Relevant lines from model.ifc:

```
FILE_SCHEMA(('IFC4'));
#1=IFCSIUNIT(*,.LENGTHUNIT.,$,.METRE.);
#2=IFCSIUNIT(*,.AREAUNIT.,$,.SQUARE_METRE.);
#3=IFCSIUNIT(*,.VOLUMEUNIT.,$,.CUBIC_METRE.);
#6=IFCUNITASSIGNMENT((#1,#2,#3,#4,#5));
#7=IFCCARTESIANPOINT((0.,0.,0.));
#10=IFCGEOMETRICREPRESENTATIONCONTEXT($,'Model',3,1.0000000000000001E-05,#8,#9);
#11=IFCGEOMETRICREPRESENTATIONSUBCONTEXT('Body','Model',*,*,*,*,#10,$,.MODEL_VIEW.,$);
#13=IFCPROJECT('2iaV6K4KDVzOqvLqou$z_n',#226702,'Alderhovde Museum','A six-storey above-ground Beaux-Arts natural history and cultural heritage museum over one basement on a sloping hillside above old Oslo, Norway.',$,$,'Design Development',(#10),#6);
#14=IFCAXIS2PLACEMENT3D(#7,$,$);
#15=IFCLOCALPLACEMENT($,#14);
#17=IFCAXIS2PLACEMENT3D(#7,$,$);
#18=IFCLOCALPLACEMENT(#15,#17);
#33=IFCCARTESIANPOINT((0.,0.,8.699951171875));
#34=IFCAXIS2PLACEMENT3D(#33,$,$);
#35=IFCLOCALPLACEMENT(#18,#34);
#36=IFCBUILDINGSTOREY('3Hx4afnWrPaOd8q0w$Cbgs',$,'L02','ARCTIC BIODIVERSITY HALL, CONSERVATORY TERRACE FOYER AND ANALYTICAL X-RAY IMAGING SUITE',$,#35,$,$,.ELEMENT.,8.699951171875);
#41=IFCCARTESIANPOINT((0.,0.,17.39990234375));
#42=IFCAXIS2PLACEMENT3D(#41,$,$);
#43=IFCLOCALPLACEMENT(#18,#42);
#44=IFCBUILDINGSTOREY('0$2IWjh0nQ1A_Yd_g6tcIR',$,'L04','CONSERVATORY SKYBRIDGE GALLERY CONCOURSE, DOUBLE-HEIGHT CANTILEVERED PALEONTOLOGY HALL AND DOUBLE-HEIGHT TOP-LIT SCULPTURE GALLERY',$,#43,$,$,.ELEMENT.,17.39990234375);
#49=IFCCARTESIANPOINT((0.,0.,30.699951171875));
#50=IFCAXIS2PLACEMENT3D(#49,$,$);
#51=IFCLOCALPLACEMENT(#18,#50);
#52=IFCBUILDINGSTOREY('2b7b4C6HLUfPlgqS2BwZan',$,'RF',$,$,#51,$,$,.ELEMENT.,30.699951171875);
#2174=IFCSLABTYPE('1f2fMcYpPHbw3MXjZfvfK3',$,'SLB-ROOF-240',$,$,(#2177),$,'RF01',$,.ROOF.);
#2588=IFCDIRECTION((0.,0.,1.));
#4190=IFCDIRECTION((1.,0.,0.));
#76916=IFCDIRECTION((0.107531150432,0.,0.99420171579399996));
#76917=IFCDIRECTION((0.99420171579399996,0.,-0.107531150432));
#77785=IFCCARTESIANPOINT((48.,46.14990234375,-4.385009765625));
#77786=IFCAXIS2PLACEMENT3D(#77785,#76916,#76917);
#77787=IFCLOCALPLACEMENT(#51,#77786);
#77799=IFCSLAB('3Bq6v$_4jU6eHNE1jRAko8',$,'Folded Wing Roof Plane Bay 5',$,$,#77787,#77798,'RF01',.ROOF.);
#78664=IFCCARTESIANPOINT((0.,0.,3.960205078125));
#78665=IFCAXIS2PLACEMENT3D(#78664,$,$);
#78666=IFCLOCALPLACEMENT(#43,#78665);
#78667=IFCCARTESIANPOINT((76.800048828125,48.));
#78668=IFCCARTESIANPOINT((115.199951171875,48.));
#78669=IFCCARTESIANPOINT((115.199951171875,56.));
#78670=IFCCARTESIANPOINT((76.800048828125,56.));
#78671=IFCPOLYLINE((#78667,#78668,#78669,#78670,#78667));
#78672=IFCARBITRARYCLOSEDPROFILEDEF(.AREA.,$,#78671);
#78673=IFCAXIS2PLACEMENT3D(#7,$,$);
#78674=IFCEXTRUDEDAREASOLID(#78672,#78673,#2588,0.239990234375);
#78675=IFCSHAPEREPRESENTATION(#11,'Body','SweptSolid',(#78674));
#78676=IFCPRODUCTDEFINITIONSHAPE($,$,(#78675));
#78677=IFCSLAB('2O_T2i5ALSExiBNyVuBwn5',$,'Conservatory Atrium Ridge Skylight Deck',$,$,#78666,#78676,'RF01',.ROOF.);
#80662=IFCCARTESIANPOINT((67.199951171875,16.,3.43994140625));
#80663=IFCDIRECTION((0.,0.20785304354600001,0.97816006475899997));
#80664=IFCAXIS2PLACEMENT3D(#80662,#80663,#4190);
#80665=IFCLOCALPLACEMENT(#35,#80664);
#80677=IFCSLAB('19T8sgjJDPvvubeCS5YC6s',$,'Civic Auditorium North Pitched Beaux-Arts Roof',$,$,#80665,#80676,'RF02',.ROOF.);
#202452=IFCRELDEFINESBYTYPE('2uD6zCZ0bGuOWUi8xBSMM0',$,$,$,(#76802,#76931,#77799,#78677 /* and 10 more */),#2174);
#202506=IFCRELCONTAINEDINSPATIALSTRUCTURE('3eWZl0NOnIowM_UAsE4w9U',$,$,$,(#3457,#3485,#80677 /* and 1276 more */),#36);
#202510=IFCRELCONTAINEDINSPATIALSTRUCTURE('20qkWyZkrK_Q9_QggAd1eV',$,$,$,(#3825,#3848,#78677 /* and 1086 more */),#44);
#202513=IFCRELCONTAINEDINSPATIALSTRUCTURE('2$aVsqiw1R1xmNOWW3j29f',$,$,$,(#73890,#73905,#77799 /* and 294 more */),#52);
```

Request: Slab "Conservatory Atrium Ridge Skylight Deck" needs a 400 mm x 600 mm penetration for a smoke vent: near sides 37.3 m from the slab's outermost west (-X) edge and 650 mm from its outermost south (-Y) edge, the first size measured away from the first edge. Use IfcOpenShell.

```python
import numpy as np
import ifcopenshell
import ifcopenshell.api.feature
import ifcopenshell.api.geometry
import ifcopenshell.api.root
import ifcopenshell.geom
import ifcopenshell.util.placement
import ifcopenshell.util.representation
import ifcopenshell.util.shape
import ifcopenshell.util.unit

model = ifcopenshell.open("model.ifc")
unit_scale = ifcopenshell.util.unit.calculate_unit_scale(model)
settings = ifcopenshell.geom.settings()


def volume(element):
    """Net volume in cubic metres, openings subtracted."""
    shape = ifcopenshell.geom.create_shape(settings, element)
    return ifcopenshell.util.shape.get_volume(shape.geometry)


slab = model.by_id(78677)
before = volume(slab)

# Extent in the slab's own axes, in metres. The edges named are its -X and -Y sides.
slab_shape = ifcopenshell.geom.create_shape(settings, slab)
vertices = ifcopenshell.util.shape.get_vertices(slab_shape.geometry)
x_min, y_min, bottom = vertices.min(axis=0)
top = vertices[:, 2].max()

opening = ifcopenshell.api.root.create_entity(model, ifc_class="IfcOpeningElement", name="Smoke vent opening", predefined_type="OPENING")
context = ifcopenshell.util.representation.get_context(model, "Model", "Body", "MODEL_VIEW")
width, depth = 0.4, 0.6
outline = [(0.0, 0.0), (width, 0.0), (width, depth), (0.0, depth), (0.0, 0.0)]
# Overshoot both faces by 50 mm so the cut is clean.
shape = ifcopenshell.api.geometry.add_slab_representation(
    model, context=context, depth=top - bottom + 0.1, polyline=outline
)
ifcopenshell.api.geometry.assign_representation(model, product=opening, representation=shape)

matrix = ifcopenshell.util.placement.get_local_placement(slab.ObjectPlacement)
matrix[:, 3] = matrix @ np.append(np.array([x_min + 37.3, y_min + 0.65, bottom - 0.05]) / unit_scale, 1.0)
ifcopenshell.api.geometry.edit_object_placement(model, product=opening, matrix=matrix, is_si=False)
ifcopenshell.api.feature.add_feature(model, feature=opening, element=slab)

after = volume(slab)

print(f"slab volume {before:.3f} -> {after:.3f} m3")

model.write("model_rev.ifc")
```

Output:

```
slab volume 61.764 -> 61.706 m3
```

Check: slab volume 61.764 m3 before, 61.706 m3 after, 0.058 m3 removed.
